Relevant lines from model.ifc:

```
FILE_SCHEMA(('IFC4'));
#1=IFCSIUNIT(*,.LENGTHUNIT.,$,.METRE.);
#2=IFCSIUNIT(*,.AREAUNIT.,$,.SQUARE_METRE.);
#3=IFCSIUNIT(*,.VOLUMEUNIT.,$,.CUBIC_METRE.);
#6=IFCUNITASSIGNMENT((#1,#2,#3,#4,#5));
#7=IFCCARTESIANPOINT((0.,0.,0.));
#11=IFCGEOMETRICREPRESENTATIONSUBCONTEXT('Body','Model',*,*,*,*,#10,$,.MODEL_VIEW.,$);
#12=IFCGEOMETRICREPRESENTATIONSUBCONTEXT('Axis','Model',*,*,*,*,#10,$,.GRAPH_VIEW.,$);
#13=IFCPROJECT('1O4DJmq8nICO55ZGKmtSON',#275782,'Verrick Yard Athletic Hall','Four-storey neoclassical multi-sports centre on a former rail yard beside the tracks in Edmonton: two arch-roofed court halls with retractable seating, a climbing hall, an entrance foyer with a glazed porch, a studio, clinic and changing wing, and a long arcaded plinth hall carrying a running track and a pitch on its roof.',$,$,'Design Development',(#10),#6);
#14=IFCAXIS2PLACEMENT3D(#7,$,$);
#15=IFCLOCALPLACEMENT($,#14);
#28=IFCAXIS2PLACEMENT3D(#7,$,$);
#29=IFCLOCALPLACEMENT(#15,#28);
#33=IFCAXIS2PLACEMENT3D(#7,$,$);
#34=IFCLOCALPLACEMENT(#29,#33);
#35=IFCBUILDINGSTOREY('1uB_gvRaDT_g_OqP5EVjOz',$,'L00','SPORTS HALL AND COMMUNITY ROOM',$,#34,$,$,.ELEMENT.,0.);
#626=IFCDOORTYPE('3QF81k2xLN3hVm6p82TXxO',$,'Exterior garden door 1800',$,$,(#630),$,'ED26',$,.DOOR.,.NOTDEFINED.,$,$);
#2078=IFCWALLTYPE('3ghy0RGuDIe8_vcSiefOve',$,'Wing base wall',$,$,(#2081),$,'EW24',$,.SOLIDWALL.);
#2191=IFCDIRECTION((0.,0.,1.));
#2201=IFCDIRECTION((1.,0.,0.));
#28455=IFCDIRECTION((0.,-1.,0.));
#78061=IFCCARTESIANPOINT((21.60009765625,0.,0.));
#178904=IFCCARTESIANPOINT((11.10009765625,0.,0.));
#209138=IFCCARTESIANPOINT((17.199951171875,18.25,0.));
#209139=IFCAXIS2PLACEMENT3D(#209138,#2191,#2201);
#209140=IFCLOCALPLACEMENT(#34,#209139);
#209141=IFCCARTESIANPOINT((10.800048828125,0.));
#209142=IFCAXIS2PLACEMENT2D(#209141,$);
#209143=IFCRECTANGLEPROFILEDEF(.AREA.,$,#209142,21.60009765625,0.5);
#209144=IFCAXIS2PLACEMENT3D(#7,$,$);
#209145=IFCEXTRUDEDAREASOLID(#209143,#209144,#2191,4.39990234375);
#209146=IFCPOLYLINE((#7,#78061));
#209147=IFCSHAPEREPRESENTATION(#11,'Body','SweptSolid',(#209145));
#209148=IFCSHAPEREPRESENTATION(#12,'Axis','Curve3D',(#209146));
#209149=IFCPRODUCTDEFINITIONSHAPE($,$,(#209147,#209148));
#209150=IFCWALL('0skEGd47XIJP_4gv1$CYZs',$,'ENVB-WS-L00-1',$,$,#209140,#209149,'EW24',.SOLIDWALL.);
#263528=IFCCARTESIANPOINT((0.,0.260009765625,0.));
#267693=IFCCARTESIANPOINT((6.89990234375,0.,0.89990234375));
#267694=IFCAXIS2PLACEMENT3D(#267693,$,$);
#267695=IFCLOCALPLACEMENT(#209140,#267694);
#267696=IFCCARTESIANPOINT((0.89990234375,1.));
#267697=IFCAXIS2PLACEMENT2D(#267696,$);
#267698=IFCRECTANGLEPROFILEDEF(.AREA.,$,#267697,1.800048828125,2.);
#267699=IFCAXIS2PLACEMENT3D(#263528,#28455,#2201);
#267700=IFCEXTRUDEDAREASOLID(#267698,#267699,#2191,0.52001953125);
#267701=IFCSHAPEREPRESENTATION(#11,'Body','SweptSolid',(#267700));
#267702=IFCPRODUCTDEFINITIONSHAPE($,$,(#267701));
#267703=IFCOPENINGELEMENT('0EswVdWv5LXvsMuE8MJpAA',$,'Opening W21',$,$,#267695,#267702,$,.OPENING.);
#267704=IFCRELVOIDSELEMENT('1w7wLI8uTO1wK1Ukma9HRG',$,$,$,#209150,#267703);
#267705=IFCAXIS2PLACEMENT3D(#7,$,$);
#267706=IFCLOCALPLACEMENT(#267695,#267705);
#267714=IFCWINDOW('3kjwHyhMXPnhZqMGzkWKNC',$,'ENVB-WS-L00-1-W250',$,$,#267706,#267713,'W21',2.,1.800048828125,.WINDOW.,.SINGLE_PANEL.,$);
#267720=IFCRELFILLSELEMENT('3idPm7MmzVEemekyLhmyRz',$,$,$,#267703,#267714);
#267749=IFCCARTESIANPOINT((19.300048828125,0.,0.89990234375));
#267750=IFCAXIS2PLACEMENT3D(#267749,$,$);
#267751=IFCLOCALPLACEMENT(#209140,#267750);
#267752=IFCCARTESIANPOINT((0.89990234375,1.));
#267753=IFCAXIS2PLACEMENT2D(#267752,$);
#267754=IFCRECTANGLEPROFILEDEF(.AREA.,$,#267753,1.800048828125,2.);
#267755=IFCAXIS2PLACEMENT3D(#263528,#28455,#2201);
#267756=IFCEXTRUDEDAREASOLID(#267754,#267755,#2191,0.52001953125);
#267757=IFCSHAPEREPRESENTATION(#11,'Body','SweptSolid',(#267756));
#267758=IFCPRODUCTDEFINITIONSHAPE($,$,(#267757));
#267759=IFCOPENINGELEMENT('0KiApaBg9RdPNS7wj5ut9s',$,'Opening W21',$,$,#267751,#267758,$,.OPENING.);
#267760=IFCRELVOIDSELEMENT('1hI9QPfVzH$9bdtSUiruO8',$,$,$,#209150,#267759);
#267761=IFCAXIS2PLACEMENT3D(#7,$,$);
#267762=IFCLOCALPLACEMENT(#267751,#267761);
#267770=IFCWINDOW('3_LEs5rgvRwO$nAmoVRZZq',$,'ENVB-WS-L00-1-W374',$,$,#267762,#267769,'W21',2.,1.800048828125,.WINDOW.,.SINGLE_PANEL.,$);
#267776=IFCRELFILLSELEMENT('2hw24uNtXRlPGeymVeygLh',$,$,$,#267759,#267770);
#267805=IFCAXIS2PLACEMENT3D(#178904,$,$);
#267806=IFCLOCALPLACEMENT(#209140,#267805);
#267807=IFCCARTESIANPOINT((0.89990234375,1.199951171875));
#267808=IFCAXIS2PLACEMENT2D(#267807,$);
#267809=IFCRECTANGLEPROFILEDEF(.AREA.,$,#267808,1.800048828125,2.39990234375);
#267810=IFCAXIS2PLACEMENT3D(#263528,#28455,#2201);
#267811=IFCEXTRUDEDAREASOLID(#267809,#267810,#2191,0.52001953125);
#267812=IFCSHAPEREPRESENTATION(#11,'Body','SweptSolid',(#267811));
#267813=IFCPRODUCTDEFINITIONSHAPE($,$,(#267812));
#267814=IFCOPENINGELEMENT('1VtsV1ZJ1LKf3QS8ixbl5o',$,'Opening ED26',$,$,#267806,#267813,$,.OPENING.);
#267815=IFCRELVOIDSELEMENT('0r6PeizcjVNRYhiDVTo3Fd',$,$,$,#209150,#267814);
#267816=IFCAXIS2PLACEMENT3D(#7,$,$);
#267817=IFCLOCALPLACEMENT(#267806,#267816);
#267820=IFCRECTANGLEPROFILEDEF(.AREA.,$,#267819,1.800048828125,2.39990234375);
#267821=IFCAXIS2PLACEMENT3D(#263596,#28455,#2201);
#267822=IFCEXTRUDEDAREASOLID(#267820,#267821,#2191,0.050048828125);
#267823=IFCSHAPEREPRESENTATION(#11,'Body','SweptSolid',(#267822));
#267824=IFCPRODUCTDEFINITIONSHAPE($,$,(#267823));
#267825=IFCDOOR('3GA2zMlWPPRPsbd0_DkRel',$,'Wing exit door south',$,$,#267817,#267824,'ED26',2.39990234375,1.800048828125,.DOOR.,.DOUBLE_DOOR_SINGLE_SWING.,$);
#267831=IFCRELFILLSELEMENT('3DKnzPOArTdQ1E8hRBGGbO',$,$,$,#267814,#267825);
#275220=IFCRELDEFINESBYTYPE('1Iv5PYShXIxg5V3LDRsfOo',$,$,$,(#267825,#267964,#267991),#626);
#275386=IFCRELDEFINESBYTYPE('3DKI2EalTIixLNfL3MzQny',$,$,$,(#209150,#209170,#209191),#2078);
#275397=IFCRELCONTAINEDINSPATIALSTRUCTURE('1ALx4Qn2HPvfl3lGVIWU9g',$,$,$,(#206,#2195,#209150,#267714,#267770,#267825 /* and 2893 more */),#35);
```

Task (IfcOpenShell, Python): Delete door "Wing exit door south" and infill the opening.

```python
import ifcopenshell
import ifcopenshell.api.feature
import ifcopenshell.api.root
import ifcopenshell.geom
import ifcopenshell.util.shape

model = ifcopenshell.open("model.ifc")
settings = ifcopenshell.geom.settings()


def volume(element):
    """Net volume in cubic metres, openings subtracted."""
    shape = ifcopenshell.geom.create_shape(settings, element)
    return ifcopenshell.util.shape.get_volume(shape.geometry)


door = model.by_guid("3GA2zMlWPPRPsbd0_DkRel")
opening = door.FillsVoids[0].RelatingOpeningElement
wall = opening.VoidsElements[0].RelatingBuildingElement
before = volume(wall)

ifcopenshell.api.root.remove_product(model, product=door)
ifcopenshell.api.feature.remove_feature(model, feature=opening)

after = volume(wall)

print(f"wall volume {before:.3f} -> {after:.3f} m3")

model.write("model_updated.ifc")
```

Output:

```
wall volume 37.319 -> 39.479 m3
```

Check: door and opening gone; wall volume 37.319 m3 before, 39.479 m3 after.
